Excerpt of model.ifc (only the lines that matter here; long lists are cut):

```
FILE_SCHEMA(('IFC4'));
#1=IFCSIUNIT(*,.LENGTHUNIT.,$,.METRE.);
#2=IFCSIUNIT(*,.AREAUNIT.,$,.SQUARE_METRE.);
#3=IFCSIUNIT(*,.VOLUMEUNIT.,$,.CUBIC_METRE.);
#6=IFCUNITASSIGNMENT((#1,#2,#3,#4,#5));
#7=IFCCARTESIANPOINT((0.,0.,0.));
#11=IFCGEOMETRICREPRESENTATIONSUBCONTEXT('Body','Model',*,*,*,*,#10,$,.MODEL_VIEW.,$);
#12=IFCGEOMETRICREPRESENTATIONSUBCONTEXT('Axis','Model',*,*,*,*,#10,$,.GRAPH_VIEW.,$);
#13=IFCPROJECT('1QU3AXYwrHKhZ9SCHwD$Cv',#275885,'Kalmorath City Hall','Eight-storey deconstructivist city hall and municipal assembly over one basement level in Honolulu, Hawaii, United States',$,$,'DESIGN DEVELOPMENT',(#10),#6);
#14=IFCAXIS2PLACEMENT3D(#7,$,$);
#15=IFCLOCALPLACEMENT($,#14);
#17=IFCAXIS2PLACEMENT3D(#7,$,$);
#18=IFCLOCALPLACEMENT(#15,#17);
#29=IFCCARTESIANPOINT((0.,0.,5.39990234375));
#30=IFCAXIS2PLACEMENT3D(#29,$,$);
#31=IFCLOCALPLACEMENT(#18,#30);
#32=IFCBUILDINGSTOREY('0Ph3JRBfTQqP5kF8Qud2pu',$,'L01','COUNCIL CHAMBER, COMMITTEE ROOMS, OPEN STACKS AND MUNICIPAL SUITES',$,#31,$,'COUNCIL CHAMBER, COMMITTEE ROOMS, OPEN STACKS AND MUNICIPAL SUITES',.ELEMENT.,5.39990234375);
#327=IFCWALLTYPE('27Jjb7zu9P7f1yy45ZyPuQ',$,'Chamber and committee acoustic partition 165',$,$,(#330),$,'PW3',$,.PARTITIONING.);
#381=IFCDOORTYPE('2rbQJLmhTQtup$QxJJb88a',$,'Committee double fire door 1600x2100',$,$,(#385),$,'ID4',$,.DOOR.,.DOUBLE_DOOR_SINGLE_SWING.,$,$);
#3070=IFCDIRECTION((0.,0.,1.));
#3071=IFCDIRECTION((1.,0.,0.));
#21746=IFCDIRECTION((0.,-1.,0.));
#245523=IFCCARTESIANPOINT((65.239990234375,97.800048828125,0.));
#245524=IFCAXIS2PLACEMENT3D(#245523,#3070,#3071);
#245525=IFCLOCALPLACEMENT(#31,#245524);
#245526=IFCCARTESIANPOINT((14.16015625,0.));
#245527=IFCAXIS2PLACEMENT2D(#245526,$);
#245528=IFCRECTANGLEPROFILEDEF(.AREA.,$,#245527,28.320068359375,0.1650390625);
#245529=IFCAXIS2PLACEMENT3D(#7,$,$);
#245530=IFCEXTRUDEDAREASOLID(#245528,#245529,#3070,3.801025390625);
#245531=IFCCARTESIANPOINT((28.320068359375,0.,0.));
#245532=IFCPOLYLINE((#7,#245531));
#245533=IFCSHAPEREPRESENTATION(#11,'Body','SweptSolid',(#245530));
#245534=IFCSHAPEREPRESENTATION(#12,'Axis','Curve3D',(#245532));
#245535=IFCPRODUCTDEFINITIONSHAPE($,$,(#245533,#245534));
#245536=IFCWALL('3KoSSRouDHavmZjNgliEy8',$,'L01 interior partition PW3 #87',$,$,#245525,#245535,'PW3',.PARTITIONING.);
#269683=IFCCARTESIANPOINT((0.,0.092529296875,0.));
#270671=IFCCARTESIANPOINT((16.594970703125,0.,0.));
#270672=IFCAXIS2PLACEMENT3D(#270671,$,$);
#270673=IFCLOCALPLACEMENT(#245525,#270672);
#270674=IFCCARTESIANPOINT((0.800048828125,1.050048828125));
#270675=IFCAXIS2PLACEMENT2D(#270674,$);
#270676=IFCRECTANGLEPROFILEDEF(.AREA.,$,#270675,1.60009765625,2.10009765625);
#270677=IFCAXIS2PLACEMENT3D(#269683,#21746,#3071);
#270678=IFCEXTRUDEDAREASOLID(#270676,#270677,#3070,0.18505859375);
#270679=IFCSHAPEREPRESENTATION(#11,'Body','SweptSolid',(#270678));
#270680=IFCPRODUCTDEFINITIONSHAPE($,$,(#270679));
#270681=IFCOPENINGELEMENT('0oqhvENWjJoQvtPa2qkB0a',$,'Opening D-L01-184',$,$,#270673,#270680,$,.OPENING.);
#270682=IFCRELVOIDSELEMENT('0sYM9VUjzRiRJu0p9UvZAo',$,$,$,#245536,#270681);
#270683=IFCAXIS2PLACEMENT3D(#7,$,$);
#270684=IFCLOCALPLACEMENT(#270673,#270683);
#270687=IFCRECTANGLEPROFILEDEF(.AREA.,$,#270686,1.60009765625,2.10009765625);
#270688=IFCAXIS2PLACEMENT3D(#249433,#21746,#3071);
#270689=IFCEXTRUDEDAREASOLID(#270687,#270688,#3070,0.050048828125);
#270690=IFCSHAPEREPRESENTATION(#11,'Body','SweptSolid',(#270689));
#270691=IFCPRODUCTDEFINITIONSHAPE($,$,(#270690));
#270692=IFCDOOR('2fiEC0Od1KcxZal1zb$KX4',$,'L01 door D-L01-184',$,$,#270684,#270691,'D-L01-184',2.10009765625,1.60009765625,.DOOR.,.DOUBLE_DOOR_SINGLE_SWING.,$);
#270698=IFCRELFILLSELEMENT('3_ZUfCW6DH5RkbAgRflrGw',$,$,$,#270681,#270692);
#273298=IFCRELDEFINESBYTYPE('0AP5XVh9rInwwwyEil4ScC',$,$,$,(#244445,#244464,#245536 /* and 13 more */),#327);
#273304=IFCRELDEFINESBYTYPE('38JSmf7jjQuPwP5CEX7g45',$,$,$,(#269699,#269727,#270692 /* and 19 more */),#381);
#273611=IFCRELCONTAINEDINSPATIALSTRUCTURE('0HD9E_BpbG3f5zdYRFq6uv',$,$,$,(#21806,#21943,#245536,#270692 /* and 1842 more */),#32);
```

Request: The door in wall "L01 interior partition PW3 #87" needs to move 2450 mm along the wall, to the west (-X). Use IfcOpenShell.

```python
import ifcopenshell
import ifcopenshell.api.geometry
import ifcopenshell.util.placement
import ifcopenshell.util.unit

model = ifcopenshell.open("model.ifc")
unit_scale = ifcopenshell.util.unit.calculate_unit_scale(model)

door = model.by_guid("2fiEC0Od1KcxZal1zb$KX4")
opening = door.FillsVoids[0].RelatingOpeningElement
wall = opening.VoidsElements[0].RelatingBuildingElement

wall_matrix = ifcopenshell.util.placement.get_local_placement(wall.ObjectPlacement)
shift = wall_matrix[:3, 0] * -2.45 / unit_scale
before = ifcopenshell.util.placement.get_local_placement(door.ObjectPlacement)[:3, 3].copy()

# The door is placed relative to its opening, so it follows when the opening moves.
matrix = ifcopenshell.util.placement.get_local_placement(opening.ObjectPlacement)
matrix[:3, 3] += shift
ifcopenshell.api.geometry.edit_object_placement(
    model, product=opening, matrix=matrix, is_si=False, should_transform_children=True
)

after = ifcopenshell.util.placement.get_local_placement(door.ObjectPlacement)[:3, 3]
print("door moved by", (after - before).round(3) + 0.0)

model.write("model_rev.ifc")
```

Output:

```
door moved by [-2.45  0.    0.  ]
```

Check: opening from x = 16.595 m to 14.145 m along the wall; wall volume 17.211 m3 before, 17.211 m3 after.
